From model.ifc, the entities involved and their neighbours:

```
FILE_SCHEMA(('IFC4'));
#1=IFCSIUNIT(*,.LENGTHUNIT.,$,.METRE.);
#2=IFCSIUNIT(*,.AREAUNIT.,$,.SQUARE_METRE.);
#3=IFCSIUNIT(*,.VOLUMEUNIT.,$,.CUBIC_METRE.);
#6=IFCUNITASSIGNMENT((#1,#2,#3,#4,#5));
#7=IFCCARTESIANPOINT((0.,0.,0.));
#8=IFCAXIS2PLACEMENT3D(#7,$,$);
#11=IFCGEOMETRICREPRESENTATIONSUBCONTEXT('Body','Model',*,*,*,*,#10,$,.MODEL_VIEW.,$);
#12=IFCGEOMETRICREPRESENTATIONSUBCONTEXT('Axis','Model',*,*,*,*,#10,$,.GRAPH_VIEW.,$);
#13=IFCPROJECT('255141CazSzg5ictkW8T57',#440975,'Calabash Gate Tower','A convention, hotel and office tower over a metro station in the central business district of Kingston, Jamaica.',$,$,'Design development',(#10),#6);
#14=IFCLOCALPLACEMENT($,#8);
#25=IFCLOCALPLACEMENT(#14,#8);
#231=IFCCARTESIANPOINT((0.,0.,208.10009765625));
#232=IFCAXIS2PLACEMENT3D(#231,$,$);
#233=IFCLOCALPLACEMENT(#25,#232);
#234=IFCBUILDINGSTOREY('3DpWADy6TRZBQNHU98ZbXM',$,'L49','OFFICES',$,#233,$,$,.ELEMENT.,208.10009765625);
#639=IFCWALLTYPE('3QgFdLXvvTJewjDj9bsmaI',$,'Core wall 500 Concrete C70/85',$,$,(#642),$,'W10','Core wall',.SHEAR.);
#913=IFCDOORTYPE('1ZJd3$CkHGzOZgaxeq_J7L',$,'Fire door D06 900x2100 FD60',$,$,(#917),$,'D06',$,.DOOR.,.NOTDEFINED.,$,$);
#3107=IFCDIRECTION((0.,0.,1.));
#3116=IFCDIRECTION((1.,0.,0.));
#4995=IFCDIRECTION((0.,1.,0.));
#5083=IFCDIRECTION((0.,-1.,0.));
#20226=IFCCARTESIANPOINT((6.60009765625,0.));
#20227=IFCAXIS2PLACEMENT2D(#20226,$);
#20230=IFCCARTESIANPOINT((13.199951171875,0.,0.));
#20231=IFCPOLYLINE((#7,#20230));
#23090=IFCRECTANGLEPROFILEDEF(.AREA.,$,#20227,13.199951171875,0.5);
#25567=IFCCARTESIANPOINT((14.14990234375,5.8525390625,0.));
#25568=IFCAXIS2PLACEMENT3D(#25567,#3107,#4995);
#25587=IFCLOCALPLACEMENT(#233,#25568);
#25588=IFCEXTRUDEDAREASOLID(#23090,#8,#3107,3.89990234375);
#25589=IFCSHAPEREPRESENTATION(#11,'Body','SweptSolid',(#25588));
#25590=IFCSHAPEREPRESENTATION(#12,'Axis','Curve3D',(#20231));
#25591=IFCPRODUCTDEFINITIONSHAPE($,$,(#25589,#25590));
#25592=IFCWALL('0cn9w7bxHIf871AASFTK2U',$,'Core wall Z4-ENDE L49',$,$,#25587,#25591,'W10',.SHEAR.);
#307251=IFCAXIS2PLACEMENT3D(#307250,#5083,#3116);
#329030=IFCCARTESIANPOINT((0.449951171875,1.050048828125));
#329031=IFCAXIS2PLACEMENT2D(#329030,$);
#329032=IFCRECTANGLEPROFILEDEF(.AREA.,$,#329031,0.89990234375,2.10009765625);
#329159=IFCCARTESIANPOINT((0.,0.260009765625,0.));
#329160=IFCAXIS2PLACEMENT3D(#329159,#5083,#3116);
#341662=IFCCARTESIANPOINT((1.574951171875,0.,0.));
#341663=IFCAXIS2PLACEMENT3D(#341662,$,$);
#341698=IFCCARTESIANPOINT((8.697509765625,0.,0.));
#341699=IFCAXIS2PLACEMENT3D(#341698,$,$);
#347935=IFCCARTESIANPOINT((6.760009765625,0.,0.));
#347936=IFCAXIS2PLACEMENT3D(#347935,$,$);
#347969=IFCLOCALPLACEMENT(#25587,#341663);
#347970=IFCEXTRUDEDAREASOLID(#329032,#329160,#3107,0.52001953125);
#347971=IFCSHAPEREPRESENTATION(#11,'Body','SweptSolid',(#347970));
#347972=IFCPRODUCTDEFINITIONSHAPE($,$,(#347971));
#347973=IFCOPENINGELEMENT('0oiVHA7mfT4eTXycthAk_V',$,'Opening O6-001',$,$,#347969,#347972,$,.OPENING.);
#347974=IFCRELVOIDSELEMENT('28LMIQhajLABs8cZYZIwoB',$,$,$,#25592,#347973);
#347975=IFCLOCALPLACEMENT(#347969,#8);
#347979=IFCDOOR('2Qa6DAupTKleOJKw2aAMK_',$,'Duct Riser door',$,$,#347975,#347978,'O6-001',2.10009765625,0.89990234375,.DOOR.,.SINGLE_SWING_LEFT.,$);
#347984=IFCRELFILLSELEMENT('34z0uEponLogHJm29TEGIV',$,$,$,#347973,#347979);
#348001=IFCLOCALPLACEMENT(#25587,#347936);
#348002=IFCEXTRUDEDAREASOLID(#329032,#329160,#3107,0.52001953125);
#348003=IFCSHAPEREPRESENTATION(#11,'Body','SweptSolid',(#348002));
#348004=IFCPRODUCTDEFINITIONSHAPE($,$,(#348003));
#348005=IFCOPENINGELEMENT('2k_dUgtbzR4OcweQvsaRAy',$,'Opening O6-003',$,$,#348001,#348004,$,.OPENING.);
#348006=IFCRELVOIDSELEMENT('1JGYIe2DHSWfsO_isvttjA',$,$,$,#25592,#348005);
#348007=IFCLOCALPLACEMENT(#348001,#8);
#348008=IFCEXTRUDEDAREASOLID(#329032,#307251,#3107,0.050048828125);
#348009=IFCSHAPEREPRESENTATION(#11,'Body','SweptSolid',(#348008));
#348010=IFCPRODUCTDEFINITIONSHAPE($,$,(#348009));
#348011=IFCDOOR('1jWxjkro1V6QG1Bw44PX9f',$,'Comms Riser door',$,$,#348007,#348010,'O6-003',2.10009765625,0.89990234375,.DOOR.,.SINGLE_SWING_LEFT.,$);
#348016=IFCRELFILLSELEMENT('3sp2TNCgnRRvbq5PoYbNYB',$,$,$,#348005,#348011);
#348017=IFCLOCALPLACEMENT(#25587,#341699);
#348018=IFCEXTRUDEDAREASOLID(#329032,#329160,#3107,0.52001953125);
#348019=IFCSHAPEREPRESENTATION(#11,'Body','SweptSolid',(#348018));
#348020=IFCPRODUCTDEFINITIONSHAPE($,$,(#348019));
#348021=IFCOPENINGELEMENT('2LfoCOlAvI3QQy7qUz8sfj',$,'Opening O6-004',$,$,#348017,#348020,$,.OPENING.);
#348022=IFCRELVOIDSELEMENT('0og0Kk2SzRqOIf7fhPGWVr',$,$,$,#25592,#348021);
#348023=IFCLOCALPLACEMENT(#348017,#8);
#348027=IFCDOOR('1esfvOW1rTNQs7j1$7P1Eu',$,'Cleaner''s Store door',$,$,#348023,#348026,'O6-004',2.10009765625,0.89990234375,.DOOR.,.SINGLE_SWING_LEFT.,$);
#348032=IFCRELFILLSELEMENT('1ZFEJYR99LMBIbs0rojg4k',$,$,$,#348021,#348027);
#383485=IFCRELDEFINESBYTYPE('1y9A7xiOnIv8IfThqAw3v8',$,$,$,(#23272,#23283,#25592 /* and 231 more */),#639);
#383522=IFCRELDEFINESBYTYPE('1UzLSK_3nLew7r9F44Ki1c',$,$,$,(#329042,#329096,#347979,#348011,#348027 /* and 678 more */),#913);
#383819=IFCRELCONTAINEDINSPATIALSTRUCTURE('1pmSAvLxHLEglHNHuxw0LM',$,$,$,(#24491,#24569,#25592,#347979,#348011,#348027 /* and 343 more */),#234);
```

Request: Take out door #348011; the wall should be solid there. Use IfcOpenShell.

```python
import ifcopenshell
import ifcopenshell.api.feature
import ifcopenshell.api.root
import ifcopenshell.geom
import ifcopenshell.util.shape

model = ifcopenshell.open("model.ifc")
settings = ifcopenshell.geom.settings()


def volume(element):
    """Net volume in cubic metres, openings subtracted."""
    shape = ifcopenshell.geom.create_shape(settings, element)
    return ifcopenshell.util.shape.get_volume(shape.geometry)


door = model.by_guid("1jWxjkro1V6QG1Bw44PX9f")
opening = door.FillsVoids[0].RelatingOpeningElement
wall = opening.VoidsElements[0].RelatingBuildingElement
before = volume(wall)

ifcopenshell.api.root.remove_product(model, product=door)
ifcopenshell.api.feature.remove_feature(model, feature=opening)

after = volume(wall)

print(f"wall volume {before:.3f} -> {after:.3f} m3")

model.write("model_edited.ifc")
```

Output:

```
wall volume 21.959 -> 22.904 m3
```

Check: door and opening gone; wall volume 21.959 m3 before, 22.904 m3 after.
